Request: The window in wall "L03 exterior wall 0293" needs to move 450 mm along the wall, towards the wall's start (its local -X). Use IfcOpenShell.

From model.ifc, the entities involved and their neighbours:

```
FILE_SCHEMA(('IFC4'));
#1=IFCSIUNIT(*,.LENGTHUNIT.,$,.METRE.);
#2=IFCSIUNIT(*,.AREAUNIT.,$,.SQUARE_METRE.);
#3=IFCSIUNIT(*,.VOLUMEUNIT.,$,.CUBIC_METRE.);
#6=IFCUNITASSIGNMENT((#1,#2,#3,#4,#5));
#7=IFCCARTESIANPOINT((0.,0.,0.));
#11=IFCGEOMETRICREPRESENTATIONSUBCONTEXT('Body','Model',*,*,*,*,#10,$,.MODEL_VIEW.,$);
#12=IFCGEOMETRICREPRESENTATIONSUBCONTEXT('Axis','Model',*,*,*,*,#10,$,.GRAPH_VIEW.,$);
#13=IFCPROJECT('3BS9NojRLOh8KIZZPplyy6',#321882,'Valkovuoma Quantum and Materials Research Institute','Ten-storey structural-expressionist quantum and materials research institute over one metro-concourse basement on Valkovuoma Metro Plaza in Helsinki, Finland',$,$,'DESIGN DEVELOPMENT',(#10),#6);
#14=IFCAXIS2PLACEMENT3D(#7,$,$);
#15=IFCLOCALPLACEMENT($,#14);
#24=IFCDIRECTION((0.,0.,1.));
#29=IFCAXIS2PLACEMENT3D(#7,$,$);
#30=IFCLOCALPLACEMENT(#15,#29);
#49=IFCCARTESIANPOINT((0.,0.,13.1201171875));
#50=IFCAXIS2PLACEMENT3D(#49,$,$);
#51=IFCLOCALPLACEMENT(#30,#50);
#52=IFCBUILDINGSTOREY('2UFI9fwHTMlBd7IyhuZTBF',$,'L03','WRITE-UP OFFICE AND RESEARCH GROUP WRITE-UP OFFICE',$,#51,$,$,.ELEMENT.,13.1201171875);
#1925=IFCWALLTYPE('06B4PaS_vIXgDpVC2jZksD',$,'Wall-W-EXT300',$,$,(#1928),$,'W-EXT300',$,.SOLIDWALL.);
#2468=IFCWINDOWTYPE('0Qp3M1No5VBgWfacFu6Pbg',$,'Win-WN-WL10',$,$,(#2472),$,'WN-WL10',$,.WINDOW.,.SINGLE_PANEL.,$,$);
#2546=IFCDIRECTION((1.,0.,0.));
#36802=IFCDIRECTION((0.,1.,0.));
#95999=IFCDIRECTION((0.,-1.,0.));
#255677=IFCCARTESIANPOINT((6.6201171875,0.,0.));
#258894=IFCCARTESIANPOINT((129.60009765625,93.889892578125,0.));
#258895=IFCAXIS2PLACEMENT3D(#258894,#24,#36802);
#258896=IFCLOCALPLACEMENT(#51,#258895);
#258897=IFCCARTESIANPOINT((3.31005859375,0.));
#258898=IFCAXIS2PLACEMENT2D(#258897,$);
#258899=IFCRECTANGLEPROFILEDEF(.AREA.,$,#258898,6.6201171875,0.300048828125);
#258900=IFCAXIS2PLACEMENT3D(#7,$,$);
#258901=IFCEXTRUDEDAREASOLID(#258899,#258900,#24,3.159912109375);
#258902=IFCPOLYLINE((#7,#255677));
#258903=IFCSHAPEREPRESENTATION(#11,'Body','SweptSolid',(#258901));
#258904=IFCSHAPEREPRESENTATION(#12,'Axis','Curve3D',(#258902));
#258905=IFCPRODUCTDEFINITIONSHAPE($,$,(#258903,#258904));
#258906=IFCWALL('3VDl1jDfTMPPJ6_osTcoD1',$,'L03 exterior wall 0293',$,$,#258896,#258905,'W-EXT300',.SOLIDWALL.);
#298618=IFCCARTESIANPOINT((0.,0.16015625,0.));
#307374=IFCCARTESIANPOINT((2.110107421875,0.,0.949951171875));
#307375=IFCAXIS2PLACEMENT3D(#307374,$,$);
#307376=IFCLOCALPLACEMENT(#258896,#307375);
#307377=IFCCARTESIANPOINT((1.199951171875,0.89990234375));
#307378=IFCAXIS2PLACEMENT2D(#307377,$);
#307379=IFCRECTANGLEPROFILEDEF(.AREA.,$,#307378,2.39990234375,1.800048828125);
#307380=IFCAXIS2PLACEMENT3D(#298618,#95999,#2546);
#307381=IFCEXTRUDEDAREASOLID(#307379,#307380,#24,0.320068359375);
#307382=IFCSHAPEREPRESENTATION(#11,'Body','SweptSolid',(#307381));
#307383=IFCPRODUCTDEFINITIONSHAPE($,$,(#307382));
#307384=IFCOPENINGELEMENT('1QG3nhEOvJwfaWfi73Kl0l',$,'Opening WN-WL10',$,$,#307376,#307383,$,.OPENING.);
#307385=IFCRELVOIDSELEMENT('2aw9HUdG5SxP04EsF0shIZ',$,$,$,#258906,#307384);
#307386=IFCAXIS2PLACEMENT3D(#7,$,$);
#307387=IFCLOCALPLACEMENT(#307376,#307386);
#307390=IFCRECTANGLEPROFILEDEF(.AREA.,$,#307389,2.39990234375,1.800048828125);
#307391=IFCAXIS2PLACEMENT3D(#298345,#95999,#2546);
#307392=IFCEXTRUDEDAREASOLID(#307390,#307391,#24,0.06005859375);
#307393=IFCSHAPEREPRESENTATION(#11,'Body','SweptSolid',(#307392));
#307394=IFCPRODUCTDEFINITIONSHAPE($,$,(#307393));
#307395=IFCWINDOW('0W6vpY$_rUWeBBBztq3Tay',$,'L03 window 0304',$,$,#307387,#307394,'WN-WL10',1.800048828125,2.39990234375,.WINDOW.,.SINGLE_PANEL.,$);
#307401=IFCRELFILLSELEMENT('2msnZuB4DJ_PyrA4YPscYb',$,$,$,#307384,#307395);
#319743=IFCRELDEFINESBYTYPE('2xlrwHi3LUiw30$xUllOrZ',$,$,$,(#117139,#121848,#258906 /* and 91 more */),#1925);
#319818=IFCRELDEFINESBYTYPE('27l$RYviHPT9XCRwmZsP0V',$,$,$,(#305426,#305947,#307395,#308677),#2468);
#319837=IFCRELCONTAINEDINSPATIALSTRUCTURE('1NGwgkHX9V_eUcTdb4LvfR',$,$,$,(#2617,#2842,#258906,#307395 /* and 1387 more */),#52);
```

```python
import ifcopenshell
import ifcopenshell.api.geometry
import ifcopenshell.util.placement

model = ifcopenshell.open("model.ifc")

window = model.by_id(307395)
opening = window.FillsVoids[0].RelatingOpeningElement
wall = opening.VoidsElements[0].RelatingBuildingElement

wall_matrix = ifcopenshell.util.placement.get_local_placement(wall.ObjectPlacement)
shift = wall_matrix[:3, 0] * -0.45
before = ifcopenshell.util.placement.get_local_placement(window.ObjectPlacement)[:3, 3].copy()

# The window is placed relative to its opening, so it follows when the opening moves.
matrix = ifcopenshell.util.placement.get_local_placement(opening.ObjectPlacement)
matrix[:3, 3] += shift
ifcopenshell.api.geometry.edit_object_placement(
    model, product=opening, matrix=matrix, is_si=False, should_transform_children=True
)

after = ifcopenshell.util.placement.get_local_placement(window.ObjectPlacement)[:3, 3]
print("window moved by", (after - before).round(3) + 0.0)

model.write("model_edited.ifc")
```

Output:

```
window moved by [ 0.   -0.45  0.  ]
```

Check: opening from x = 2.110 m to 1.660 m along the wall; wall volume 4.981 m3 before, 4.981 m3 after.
